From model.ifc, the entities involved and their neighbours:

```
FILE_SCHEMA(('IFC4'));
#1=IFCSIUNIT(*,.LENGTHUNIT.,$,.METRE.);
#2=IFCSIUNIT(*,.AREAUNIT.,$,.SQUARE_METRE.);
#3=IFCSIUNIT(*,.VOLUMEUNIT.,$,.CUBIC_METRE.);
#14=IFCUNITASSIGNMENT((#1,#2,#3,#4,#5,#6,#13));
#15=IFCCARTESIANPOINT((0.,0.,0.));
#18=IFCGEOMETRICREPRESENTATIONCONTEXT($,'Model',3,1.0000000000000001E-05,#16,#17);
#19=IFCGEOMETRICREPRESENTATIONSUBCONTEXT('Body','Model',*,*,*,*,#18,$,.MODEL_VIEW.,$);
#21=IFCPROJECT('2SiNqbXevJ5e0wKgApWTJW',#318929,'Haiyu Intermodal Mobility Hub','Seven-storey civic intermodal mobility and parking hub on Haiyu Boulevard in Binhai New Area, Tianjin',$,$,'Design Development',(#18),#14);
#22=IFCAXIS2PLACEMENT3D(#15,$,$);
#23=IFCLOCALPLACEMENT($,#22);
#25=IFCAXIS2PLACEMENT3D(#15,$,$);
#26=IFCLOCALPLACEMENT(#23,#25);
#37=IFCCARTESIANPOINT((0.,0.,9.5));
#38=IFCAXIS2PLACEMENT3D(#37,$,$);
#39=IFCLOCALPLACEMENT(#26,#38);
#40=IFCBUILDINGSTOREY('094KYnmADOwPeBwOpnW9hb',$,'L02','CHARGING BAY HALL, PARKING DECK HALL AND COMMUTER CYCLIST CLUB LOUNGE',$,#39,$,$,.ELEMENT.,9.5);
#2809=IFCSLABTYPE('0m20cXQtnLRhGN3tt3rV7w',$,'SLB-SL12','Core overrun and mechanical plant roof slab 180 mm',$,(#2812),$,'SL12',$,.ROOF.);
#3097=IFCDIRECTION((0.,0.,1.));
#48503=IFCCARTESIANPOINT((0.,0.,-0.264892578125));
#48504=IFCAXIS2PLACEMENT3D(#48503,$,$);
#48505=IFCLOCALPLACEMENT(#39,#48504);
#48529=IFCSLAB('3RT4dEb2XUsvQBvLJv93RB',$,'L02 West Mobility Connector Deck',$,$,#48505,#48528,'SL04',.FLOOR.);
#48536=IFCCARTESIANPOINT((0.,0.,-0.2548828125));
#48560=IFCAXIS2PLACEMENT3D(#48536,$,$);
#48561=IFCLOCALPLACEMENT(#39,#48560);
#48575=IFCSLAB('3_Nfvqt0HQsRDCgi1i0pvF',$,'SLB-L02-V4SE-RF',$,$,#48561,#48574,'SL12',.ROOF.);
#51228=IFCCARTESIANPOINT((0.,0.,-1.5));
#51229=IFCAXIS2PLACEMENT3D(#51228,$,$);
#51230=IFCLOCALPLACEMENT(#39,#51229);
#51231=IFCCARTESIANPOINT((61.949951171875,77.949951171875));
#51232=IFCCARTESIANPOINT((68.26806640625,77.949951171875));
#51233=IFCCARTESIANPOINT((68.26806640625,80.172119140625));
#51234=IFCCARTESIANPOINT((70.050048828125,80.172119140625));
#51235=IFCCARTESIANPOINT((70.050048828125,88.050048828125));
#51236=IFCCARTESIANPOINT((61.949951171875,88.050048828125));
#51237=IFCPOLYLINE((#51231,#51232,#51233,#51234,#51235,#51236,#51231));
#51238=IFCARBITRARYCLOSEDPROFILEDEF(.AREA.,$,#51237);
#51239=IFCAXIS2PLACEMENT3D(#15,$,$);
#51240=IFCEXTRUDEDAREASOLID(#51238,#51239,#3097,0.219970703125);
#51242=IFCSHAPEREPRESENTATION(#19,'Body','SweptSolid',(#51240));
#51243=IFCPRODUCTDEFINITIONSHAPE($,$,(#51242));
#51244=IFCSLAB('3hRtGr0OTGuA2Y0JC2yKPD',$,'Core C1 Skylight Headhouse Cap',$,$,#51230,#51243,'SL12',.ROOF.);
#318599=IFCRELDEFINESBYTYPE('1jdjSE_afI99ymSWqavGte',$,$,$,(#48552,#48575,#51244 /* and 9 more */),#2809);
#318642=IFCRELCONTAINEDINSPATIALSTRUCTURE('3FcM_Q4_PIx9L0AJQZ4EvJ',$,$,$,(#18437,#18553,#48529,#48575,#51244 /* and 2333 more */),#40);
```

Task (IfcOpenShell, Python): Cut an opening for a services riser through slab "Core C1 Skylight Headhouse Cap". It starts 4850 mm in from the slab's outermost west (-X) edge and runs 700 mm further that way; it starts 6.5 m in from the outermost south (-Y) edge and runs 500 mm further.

```python
import numpy as np
import ifcopenshell
import ifcopenshell.api.feature
import ifcopenshell.api.geometry
import ifcopenshell.api.root
import ifcopenshell.geom
import ifcopenshell.util.placement
import ifcopenshell.util.representation
import ifcopenshell.util.shape
import ifcopenshell.util.unit

model = ifcopenshell.open("model.ifc")
unit_scale = ifcopenshell.util.unit.calculate_unit_scale(model)
settings = ifcopenshell.geom.settings()


def volume(element):
    """Net volume in cubic metres, openings subtracted."""
    shape = ifcopenshell.geom.create_shape(settings, element)
    return ifcopenshell.util.shape.get_volume(shape.geometry)


slab = model.by_id(51244)
before = volume(slab)

# Extent in the slab's own axes, in metres. The edges named are its -X and -Y sides.
slab_shape = ifcopenshell.geom.create_shape(settings, slab)
vertices = ifcopenshell.util.shape.get_vertices(slab_shape.geometry)
x_min, y_min, bottom = vertices.min(axis=0)
top = vertices[:, 2].max()

opening = ifcopenshell.api.root.create_entity(model, ifc_class="IfcOpeningElement", name="Services riser opening", predefined_type="OPENING")
context = ifcopenshell.util.representation.get_context(model, "Model", "Body", "MODEL_VIEW")
width, depth = 0.7, 0.5
outline = [(0.0, 0.0), (width, 0.0), (width, depth), (0.0, depth), (0.0, 0.0)]
# Overshoot both faces by 50 mm so the cut is clean.
shape = ifcopenshell.api.geometry.add_slab_representation(
    model, context=context, depth=top - bottom + 0.1, polyline=outline
)
ifcopenshell.api.geometry.assign_representation(model, product=opening, representation=shape)

matrix = ifcopenshell.util.placement.get_local_placement(slab.ObjectPlacement)
matrix[:, 3] = matrix @ np.append(np.array([x_min + 4.85, y_min + 6.5, bottom - 0.05]) / unit_scale, 1.0)
ifcopenshell.api.geometry.edit_object_placement(model, product=opening, matrix=matrix, is_si=False)
ifcopenshell.api.feature.add_feature(model, feature=opening, element=slab)

after = volume(slab)

print(f"slab volume {before:.3f} -> {after:.3f} m3")

model.write("model_updated.ifc")
```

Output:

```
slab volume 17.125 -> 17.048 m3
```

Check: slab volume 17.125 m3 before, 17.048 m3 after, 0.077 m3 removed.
